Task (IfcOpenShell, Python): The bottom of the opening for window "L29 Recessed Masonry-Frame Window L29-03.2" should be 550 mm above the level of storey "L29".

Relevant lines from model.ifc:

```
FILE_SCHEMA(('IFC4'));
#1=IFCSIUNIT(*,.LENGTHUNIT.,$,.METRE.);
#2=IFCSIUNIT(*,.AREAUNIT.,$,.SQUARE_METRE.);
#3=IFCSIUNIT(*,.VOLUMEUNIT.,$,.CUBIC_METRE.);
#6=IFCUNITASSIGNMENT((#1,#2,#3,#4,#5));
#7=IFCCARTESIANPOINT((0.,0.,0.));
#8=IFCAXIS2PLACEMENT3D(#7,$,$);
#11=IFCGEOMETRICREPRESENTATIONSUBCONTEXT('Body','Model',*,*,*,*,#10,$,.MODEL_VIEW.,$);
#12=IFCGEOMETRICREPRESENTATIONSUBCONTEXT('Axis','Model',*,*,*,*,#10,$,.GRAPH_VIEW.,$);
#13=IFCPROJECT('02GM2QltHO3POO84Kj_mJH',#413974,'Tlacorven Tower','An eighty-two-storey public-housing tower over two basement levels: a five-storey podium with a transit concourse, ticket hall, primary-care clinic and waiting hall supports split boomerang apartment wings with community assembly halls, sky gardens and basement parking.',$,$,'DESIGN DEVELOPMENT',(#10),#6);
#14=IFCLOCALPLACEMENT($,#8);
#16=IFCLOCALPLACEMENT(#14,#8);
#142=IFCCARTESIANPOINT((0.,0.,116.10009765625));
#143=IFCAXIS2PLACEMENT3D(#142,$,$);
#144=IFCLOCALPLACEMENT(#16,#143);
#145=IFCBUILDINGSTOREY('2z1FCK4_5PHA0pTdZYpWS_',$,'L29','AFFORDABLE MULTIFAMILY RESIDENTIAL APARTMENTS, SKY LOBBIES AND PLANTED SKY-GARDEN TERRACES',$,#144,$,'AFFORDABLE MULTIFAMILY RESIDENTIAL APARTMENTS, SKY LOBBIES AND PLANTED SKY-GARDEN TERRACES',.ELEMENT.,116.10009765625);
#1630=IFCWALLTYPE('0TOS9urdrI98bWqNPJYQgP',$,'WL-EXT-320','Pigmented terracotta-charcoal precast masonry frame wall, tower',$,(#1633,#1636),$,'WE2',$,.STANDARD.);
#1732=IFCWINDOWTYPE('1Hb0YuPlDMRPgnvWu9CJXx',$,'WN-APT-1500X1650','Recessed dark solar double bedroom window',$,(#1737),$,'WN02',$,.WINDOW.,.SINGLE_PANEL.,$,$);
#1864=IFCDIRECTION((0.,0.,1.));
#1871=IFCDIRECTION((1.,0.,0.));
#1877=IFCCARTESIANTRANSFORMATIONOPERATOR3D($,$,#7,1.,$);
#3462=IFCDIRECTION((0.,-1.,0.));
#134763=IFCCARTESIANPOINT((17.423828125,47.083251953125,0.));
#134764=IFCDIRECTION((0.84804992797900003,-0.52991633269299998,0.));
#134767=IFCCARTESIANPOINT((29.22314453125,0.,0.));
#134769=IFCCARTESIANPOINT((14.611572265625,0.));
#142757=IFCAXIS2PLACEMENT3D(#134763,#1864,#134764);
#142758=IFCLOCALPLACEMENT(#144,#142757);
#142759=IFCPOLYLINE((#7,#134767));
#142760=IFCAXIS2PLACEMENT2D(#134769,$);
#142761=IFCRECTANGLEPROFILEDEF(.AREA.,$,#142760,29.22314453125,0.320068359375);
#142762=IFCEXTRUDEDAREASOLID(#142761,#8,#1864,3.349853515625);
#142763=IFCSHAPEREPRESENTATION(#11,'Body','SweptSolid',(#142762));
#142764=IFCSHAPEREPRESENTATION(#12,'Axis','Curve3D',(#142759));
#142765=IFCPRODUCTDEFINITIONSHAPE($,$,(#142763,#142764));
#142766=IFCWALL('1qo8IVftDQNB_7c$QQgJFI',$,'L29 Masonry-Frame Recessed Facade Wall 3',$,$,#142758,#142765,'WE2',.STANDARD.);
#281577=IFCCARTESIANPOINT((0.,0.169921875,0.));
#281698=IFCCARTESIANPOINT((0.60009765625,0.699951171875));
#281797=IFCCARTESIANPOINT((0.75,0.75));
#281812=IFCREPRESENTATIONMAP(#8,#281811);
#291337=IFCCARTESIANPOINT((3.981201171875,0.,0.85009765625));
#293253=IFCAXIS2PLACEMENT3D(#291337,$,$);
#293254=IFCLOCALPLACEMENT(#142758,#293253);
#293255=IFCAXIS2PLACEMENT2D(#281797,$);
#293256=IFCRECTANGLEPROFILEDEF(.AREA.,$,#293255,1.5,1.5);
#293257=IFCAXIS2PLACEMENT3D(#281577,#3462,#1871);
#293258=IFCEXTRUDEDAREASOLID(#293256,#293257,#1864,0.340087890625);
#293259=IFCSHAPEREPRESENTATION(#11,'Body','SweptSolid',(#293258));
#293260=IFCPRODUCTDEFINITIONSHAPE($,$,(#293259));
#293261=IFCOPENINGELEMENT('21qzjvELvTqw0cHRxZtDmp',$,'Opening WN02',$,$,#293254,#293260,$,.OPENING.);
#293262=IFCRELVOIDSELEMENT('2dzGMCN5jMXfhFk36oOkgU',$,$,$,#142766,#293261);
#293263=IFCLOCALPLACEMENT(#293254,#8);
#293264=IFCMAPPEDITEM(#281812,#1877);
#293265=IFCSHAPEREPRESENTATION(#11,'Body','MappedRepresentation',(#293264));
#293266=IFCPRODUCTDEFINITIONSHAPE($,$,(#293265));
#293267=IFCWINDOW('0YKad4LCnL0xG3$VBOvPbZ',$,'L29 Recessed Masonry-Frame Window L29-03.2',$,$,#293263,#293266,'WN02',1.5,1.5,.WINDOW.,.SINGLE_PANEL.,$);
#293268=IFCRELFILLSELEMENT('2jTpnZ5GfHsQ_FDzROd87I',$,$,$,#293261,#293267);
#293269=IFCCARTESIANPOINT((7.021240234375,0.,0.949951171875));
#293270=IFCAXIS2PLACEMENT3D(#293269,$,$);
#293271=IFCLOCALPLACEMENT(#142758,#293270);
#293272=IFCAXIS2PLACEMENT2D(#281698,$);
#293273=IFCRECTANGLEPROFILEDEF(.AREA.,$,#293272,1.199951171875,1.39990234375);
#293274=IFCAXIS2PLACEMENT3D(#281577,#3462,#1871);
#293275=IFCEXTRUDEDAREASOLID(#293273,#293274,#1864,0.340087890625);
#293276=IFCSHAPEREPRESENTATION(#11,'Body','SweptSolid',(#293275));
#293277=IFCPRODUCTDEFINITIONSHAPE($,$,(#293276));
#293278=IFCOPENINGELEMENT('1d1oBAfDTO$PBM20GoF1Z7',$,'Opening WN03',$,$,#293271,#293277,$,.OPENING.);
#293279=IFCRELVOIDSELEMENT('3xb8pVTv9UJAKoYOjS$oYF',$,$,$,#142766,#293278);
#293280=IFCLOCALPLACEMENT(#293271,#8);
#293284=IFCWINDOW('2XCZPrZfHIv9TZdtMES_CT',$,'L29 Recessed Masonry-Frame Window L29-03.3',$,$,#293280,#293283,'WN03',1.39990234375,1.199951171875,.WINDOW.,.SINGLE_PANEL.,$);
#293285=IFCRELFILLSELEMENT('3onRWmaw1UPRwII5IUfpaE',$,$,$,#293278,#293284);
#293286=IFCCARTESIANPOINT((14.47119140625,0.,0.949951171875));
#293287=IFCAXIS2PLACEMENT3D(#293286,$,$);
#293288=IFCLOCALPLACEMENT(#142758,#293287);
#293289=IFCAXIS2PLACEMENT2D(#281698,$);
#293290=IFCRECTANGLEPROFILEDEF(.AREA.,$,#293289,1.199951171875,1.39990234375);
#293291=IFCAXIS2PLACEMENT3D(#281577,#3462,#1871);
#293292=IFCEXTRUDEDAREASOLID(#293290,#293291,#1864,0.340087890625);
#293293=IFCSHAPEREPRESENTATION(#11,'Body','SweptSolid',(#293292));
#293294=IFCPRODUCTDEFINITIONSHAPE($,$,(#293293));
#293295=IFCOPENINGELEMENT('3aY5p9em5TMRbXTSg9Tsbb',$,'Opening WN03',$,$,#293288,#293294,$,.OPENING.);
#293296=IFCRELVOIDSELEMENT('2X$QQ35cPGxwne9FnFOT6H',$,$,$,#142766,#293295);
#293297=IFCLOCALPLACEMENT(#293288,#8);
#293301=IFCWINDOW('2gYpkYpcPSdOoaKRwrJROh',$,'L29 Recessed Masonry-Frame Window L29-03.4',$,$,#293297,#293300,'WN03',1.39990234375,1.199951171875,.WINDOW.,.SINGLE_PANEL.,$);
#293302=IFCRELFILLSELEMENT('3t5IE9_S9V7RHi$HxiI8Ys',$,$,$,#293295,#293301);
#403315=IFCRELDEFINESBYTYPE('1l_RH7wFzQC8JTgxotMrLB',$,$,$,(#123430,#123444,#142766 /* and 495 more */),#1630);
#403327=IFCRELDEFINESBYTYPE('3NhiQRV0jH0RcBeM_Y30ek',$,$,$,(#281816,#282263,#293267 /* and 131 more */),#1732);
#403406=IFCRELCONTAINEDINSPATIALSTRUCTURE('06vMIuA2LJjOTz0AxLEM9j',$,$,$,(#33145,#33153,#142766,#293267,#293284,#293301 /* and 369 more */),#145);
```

```python
import numpy as np
import ifcopenshell
import ifcopenshell.api.geometry
import ifcopenshell.geom
import ifcopenshell.util.element
import ifcopenshell.util.placement
import ifcopenshell.util.shape
import ifcopenshell.util.unit

model = ifcopenshell.open("model.ifc")
unit_scale = ifcopenshell.util.unit.calculate_unit_scale(model)

window = model.by_id(293267)
opening = window.FillsVoids[0].RelatingOpeningElement
storey = ifcopenshell.util.element.get_container(window, ifc_class="IfcBuildingStorey")
level = ifcopenshell.util.placement.get_local_placement(storey.ObjectPlacement)[2, 3]

# The opening's origin need not be at the sill, so measure its lowest point.
shape = ifcopenshell.geom.create_shape(ifcopenshell.geom.settings(), opening)
bottom = ifcopenshell.util.shape.get_shape_bottom_elevation(shape, shape.geometry) / unit_scale
dz = level + 0.55 / unit_scale - bottom

shift = np.array([0.0, 0.0, dz])
# The window is placed relative to its opening, so it follows when the opening moves.
matrix = ifcopenshell.util.placement.get_local_placement(opening.ObjectPlacement)
matrix[:3, 3] += shift
ifcopenshell.api.geometry.edit_object_placement(
    model, product=opening, matrix=matrix, is_si=False, should_transform_children=True
)

print(f"moved by {dz * unit_scale:+.3f} m")

model.write("model_edited.ifc")
```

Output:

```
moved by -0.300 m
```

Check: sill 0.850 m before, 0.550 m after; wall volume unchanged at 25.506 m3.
